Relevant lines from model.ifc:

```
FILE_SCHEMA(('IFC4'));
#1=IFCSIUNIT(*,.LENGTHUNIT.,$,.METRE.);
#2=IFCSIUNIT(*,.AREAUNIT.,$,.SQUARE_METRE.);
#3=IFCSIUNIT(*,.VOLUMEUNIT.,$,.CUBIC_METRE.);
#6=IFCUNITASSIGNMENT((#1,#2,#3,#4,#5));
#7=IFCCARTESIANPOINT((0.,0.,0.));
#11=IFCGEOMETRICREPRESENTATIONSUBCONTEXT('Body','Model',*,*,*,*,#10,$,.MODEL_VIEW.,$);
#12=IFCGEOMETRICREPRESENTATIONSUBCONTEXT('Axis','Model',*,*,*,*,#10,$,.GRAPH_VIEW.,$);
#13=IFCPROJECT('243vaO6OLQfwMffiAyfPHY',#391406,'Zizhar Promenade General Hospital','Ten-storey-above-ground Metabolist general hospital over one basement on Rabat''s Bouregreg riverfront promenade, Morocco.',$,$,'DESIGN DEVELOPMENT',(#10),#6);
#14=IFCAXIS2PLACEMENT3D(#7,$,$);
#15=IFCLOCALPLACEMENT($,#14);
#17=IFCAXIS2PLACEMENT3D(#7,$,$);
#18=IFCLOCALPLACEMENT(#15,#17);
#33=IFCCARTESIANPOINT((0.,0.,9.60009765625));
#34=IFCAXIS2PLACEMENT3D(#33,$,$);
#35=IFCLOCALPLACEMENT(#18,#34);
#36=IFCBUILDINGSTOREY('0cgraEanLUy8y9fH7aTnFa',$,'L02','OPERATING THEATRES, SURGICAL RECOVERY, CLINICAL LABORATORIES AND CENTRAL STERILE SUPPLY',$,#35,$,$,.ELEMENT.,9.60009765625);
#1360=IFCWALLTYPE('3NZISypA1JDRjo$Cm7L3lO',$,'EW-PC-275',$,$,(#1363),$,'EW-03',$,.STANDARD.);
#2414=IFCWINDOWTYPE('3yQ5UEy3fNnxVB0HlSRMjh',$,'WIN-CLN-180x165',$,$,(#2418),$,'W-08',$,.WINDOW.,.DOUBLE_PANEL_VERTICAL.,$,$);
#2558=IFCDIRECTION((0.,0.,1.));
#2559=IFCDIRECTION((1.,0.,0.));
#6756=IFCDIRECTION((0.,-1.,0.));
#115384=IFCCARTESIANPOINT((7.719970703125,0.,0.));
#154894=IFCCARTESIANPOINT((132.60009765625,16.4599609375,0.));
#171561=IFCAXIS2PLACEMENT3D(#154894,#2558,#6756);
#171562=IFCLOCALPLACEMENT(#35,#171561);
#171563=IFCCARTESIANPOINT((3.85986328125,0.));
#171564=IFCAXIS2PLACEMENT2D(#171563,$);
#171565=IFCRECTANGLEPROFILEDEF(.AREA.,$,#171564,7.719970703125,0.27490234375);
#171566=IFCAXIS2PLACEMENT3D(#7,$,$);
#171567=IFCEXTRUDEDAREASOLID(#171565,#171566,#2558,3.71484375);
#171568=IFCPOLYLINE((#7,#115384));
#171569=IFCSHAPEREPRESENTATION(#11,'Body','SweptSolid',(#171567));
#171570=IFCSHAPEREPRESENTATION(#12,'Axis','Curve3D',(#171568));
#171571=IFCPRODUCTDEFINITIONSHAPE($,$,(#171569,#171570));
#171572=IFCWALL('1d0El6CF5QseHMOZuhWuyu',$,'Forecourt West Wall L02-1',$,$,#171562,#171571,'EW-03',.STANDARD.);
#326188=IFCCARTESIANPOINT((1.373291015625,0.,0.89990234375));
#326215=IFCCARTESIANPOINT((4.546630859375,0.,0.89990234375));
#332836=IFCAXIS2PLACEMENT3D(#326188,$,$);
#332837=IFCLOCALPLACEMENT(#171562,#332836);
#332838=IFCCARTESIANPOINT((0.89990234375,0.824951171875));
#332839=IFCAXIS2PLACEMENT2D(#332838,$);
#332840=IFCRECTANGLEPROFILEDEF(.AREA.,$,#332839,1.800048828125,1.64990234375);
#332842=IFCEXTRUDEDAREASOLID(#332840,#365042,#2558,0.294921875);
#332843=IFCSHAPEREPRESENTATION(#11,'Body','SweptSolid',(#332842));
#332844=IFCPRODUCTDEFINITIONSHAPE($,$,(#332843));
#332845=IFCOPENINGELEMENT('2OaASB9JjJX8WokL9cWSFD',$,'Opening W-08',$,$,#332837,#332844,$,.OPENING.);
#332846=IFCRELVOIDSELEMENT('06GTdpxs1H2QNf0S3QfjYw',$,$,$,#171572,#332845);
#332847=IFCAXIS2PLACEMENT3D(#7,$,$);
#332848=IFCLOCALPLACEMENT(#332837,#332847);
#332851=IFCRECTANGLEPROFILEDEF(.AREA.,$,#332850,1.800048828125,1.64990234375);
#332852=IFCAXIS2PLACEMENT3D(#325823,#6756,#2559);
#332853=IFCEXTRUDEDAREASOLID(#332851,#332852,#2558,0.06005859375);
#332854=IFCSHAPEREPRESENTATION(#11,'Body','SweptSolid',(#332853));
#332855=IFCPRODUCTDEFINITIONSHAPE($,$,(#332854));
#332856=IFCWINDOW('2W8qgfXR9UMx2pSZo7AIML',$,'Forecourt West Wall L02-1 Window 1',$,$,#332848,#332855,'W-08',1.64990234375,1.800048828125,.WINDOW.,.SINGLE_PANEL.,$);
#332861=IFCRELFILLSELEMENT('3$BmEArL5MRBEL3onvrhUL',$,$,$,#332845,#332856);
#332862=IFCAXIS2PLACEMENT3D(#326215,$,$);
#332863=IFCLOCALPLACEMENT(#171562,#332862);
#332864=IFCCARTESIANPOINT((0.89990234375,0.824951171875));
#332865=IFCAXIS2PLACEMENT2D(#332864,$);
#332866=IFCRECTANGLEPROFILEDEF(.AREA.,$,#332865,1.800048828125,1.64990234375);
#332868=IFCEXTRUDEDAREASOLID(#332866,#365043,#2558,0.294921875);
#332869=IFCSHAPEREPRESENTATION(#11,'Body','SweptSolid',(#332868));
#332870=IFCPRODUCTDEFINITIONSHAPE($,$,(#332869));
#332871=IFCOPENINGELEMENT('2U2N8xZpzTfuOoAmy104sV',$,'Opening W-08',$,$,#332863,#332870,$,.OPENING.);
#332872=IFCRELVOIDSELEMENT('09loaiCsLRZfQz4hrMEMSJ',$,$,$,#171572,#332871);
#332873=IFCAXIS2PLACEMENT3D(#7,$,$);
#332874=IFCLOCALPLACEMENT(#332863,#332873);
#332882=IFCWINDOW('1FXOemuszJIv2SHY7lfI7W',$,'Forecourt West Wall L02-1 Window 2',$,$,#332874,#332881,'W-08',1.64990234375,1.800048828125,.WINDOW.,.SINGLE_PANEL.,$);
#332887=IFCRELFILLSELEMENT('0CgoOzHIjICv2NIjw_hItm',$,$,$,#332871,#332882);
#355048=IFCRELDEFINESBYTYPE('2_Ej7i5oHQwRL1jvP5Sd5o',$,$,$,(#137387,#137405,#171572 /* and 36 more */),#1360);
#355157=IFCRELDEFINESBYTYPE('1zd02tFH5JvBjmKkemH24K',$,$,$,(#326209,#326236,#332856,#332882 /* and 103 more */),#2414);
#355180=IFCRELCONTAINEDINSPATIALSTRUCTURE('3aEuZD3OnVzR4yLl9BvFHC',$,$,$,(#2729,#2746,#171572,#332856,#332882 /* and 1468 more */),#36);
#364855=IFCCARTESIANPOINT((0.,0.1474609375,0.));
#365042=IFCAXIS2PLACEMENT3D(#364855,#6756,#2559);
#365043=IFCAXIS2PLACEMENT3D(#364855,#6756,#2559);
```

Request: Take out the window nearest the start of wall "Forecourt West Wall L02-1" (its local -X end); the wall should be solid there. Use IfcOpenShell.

```python
import ifcopenshell
import ifcopenshell.api.feature
import ifcopenshell.api.root
import ifcopenshell.geom
import ifcopenshell.util.shape

model = ifcopenshell.open("model.ifc")
settings = ifcopenshell.geom.settings()


def volume(element):
    """Net volume in cubic metres, openings subtracted."""
    shape = ifcopenshell.geom.create_shape(settings, element)
    return ifcopenshell.util.shape.get_volume(shape.geometry)


window = model.by_guid("2W8qgfXR9UMx2pSZo7AIML")
opening = window.FillsVoids[0].RelatingOpeningElement
wall = opening.VoidsElements[0].RelatingBuildingElement
before = volume(wall)

ifcopenshell.api.root.remove_product(model, product=window)
ifcopenshell.api.feature.remove_feature(model, feature=opening)

after = volume(wall)

print(f"wall volume {before:.3f} -> {after:.3f} m3")

model.write("model_updated.ifc")
```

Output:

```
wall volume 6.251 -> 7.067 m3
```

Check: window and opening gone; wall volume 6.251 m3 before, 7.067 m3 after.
